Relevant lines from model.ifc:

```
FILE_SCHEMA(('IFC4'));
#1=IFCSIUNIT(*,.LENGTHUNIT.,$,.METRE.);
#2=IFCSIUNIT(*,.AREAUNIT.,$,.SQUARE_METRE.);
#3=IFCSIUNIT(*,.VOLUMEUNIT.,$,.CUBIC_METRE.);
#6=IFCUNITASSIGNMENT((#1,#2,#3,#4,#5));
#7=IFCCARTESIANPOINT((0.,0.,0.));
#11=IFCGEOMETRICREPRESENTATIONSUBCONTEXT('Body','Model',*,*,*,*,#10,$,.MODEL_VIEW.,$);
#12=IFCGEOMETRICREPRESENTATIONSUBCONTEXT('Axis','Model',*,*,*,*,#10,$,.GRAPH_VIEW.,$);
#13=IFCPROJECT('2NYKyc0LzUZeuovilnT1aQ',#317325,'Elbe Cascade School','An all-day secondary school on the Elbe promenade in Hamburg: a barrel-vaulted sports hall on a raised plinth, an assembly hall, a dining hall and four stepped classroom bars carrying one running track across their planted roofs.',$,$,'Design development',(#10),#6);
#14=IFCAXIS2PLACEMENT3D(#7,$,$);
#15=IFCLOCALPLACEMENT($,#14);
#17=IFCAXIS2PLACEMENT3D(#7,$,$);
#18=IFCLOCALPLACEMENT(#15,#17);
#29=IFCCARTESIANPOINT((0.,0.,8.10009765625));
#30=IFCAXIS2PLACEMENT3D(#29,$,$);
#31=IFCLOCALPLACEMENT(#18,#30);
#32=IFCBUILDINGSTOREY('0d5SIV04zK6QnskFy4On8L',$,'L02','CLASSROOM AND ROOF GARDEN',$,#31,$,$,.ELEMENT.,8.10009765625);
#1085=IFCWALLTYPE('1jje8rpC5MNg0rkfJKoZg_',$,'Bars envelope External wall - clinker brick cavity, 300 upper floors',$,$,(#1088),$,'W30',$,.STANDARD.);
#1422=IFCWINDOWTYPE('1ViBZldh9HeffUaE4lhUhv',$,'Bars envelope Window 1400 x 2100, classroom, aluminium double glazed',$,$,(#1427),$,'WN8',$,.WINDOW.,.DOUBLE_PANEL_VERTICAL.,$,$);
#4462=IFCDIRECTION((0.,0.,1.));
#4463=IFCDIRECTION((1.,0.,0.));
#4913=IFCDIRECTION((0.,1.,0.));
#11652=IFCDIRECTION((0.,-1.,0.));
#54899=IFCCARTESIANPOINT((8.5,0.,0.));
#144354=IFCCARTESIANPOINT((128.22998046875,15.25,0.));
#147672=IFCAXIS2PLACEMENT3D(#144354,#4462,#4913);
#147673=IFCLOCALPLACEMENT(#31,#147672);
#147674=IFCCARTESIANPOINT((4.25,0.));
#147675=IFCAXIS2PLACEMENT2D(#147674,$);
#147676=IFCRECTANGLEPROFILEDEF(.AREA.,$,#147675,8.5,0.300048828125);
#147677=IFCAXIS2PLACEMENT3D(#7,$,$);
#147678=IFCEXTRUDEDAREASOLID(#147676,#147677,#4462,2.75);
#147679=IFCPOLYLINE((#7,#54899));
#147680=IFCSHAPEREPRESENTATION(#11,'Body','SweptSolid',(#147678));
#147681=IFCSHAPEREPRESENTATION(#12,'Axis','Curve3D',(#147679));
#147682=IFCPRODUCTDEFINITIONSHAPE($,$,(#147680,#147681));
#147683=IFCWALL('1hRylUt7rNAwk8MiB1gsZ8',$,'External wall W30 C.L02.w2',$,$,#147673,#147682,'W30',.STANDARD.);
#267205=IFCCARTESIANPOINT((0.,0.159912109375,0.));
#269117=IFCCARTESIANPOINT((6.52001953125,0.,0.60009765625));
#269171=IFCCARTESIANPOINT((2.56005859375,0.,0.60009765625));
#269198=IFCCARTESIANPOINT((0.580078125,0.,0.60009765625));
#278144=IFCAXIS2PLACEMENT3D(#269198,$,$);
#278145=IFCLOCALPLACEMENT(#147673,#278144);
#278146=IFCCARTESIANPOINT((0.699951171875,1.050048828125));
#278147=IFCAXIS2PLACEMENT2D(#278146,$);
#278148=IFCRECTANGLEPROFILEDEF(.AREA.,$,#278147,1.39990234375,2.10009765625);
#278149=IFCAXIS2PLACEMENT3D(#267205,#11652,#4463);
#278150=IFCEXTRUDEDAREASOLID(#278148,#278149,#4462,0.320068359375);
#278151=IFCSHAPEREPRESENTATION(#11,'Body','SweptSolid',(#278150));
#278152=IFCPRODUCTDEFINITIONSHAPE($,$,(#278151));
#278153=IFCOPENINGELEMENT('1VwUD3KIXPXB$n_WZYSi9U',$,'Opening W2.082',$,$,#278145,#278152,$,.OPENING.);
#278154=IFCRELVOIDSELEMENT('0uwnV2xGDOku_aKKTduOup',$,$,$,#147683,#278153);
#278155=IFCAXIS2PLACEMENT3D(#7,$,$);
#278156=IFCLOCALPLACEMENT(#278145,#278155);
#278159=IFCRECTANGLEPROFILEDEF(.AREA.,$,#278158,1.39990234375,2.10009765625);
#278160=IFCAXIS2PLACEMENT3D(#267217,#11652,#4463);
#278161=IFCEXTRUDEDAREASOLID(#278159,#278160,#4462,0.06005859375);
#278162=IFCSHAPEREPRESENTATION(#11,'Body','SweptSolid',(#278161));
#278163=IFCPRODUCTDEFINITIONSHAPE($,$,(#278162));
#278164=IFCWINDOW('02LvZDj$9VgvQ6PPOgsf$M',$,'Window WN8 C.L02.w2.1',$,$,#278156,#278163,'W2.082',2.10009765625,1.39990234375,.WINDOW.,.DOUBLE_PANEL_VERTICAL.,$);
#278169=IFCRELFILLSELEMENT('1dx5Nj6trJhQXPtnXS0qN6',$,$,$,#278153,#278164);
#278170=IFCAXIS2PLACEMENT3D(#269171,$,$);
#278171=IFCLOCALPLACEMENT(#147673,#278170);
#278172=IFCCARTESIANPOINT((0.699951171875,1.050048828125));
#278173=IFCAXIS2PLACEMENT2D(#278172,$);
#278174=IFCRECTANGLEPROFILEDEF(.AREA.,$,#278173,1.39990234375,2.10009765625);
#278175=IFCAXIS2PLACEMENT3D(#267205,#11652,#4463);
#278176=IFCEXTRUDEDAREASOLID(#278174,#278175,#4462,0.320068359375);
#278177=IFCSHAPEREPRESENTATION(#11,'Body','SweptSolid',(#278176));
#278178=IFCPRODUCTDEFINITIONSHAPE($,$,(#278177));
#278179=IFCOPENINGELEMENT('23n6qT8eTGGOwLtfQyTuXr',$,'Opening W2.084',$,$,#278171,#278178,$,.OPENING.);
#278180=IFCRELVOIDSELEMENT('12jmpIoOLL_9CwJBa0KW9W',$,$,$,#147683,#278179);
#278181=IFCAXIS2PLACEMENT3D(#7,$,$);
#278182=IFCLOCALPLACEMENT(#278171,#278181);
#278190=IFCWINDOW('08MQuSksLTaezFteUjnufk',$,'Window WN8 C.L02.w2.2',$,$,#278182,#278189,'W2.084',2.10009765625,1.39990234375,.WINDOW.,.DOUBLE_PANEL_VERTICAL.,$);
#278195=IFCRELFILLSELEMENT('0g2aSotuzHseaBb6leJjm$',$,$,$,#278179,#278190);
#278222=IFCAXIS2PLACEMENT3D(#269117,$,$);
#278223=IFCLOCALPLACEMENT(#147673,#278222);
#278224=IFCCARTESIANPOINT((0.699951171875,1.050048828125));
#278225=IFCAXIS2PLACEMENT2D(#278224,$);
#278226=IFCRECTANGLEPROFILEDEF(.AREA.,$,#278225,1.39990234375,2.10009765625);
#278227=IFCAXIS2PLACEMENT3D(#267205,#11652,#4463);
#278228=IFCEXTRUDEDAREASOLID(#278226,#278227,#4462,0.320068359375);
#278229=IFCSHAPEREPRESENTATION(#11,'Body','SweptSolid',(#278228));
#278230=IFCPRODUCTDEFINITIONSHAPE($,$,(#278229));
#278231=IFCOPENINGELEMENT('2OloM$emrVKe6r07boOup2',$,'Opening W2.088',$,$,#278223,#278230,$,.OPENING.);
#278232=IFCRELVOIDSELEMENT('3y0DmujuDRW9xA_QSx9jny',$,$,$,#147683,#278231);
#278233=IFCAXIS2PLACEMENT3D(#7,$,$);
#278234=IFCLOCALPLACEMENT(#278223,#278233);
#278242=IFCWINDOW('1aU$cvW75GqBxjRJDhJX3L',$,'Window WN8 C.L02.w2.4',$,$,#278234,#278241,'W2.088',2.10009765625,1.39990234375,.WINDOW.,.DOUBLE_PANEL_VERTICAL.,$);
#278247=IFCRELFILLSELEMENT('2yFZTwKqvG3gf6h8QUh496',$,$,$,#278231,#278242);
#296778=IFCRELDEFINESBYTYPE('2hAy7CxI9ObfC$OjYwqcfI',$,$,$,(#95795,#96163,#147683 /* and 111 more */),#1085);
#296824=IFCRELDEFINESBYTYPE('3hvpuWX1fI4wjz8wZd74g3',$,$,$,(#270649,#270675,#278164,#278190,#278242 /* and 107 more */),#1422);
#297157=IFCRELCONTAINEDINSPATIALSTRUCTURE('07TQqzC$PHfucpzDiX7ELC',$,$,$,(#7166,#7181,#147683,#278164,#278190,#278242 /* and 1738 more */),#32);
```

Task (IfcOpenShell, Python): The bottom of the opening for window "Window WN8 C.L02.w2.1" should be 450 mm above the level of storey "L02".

```python
import numpy as np
import ifcopenshell
import ifcopenshell.api.geometry
import ifcopenshell.geom
import ifcopenshell.util.element
import ifcopenshell.util.placement
import ifcopenshell.util.shape
import ifcopenshell.util.unit

model = ifcopenshell.open("model.ifc")
unit_scale = ifcopenshell.util.unit.calculate_unit_scale(model)

window = model.by_guid("02LvZDj$9VgvQ6PPOgsf$M")
opening = window.FillsVoids[0].RelatingOpeningElement
storey = ifcopenshell.util.element.get_container(window, ifc_class="IfcBuildingStorey")
level = ifcopenshell.util.placement.get_local_placement(storey.ObjectPlacement)[2, 3]

# The opening's origin need not be at the sill, so measure its lowest point.
shape = ifcopenshell.geom.create_shape(ifcopenshell.geom.settings(), opening)
bottom = ifcopenshell.util.shape.get_shape_bottom_elevation(shape, shape.geometry) / unit_scale
dz = level + 0.45 / unit_scale - bottom

shift = np.array([0.0, 0.0, dz])
# The window is placed relative to its opening, so it follows when the opening moves.
matrix = ifcopenshell.util.placement.get_local_placement(opening.ObjectPlacement)
matrix[:3, 3] += shift
ifcopenshell.api.geometry.edit_object_placement(
    model, product=opening, matrix=matrix, is_si=False, should_transform_children=True
)

print(f"moved by {dz * unit_scale:+.3f} m")

model.write("model_rev.ifc")
```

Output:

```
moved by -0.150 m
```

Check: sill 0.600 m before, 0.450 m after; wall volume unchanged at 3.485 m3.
